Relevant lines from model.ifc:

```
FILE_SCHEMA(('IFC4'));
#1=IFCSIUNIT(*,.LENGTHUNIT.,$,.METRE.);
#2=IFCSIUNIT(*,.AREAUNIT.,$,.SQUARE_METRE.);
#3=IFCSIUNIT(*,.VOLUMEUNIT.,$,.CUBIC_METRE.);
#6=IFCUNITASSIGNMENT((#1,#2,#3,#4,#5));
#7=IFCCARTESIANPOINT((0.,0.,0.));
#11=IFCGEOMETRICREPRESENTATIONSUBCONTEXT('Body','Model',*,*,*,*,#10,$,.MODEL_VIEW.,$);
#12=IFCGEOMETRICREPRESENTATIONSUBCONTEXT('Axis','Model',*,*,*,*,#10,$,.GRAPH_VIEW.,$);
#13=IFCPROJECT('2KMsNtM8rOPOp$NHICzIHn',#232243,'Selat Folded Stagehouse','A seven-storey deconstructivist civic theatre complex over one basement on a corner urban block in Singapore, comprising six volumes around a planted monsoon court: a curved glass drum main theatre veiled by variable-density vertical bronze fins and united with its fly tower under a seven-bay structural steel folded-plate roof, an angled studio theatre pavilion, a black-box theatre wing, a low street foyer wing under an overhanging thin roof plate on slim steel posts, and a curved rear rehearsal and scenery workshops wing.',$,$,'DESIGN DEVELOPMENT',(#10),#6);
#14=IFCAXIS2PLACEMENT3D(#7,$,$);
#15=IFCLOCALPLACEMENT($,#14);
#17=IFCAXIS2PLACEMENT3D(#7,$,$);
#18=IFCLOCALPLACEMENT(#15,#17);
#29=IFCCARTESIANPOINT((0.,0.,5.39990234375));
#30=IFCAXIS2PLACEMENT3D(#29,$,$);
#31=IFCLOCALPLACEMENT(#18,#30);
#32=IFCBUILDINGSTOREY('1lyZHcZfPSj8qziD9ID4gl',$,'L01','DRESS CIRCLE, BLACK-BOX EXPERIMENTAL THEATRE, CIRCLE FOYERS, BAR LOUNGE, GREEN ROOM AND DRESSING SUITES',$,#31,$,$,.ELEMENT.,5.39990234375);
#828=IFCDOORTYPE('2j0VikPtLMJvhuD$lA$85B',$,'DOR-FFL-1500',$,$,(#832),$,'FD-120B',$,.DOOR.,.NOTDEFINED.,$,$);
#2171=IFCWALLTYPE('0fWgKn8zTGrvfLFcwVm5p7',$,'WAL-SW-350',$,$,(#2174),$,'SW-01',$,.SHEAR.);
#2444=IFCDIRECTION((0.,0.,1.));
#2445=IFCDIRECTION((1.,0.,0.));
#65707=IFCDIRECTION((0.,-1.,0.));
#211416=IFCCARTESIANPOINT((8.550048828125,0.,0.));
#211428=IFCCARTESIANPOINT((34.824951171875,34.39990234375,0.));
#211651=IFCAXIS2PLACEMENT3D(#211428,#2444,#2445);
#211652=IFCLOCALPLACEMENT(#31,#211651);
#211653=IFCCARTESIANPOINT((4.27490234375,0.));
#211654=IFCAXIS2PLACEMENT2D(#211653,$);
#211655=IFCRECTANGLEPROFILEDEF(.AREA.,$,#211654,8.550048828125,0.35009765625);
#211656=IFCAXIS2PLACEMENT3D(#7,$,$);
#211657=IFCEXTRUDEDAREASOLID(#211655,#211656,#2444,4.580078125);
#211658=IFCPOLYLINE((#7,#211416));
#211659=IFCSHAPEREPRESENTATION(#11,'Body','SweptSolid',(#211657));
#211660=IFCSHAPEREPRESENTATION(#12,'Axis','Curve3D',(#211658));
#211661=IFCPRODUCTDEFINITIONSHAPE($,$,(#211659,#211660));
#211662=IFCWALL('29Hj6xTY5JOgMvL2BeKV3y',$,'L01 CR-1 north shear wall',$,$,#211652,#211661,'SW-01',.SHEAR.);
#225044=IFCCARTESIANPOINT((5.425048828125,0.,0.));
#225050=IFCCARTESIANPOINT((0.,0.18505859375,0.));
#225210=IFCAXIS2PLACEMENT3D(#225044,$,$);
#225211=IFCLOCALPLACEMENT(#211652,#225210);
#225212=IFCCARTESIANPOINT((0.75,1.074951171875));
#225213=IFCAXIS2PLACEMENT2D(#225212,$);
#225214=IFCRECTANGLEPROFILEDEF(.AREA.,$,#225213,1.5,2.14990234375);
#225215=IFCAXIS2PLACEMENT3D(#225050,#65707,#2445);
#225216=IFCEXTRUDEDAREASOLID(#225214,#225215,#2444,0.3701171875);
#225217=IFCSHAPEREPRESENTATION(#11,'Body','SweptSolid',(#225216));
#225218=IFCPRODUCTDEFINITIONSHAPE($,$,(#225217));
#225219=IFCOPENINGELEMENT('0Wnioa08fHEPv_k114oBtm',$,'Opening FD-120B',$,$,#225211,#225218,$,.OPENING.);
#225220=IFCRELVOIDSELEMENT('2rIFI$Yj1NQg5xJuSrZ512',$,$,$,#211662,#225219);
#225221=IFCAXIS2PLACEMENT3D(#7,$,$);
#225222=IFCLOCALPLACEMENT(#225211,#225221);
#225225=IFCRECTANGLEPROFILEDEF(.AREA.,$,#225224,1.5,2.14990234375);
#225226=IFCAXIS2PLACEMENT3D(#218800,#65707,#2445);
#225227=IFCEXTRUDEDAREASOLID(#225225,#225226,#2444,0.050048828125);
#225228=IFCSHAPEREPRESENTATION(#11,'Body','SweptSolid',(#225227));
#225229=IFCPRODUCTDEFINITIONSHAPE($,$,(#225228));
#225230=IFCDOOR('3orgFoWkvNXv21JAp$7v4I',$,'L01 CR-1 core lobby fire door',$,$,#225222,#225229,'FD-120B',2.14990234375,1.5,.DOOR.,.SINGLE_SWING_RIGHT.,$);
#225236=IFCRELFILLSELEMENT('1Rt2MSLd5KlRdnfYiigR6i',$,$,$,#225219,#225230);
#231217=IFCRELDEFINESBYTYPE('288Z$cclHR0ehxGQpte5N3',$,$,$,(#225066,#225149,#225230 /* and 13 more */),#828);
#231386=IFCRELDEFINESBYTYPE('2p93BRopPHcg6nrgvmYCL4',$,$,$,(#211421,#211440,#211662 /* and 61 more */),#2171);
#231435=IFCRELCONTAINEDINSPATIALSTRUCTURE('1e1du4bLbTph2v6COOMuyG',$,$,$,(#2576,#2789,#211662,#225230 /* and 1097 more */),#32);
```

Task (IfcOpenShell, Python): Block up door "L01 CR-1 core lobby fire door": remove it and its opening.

```python
import ifcopenshell
import ifcopenshell.api.feature
import ifcopenshell.api.root
import ifcopenshell.geom
import ifcopenshell.util.shape

model = ifcopenshell.open("model.ifc")
settings = ifcopenshell.geom.settings()


def volume(element):
    """Net volume in cubic metres, openings subtracted."""
    shape = ifcopenshell.geom.create_shape(settings, element)
    return ifcopenshell.util.shape.get_volume(shape.geometry)


door = model.by_guid("3orgFoWkvNXv21JAp$7v4I")
opening = door.FillsVoids[0].RelatingOpeningElement
wall = opening.VoidsElements[0].RelatingBuildingElement
before = volume(wall)

ifcopenshell.api.root.remove_product(model, product=door)
ifcopenshell.api.feature.remove_feature(model, feature=opening)

after = volume(wall)

print(f"wall volume {before:.3f} -> {after:.3f} m3")

model.write("model_updated.ifc")
```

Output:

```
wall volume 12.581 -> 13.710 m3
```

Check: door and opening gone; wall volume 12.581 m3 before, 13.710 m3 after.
